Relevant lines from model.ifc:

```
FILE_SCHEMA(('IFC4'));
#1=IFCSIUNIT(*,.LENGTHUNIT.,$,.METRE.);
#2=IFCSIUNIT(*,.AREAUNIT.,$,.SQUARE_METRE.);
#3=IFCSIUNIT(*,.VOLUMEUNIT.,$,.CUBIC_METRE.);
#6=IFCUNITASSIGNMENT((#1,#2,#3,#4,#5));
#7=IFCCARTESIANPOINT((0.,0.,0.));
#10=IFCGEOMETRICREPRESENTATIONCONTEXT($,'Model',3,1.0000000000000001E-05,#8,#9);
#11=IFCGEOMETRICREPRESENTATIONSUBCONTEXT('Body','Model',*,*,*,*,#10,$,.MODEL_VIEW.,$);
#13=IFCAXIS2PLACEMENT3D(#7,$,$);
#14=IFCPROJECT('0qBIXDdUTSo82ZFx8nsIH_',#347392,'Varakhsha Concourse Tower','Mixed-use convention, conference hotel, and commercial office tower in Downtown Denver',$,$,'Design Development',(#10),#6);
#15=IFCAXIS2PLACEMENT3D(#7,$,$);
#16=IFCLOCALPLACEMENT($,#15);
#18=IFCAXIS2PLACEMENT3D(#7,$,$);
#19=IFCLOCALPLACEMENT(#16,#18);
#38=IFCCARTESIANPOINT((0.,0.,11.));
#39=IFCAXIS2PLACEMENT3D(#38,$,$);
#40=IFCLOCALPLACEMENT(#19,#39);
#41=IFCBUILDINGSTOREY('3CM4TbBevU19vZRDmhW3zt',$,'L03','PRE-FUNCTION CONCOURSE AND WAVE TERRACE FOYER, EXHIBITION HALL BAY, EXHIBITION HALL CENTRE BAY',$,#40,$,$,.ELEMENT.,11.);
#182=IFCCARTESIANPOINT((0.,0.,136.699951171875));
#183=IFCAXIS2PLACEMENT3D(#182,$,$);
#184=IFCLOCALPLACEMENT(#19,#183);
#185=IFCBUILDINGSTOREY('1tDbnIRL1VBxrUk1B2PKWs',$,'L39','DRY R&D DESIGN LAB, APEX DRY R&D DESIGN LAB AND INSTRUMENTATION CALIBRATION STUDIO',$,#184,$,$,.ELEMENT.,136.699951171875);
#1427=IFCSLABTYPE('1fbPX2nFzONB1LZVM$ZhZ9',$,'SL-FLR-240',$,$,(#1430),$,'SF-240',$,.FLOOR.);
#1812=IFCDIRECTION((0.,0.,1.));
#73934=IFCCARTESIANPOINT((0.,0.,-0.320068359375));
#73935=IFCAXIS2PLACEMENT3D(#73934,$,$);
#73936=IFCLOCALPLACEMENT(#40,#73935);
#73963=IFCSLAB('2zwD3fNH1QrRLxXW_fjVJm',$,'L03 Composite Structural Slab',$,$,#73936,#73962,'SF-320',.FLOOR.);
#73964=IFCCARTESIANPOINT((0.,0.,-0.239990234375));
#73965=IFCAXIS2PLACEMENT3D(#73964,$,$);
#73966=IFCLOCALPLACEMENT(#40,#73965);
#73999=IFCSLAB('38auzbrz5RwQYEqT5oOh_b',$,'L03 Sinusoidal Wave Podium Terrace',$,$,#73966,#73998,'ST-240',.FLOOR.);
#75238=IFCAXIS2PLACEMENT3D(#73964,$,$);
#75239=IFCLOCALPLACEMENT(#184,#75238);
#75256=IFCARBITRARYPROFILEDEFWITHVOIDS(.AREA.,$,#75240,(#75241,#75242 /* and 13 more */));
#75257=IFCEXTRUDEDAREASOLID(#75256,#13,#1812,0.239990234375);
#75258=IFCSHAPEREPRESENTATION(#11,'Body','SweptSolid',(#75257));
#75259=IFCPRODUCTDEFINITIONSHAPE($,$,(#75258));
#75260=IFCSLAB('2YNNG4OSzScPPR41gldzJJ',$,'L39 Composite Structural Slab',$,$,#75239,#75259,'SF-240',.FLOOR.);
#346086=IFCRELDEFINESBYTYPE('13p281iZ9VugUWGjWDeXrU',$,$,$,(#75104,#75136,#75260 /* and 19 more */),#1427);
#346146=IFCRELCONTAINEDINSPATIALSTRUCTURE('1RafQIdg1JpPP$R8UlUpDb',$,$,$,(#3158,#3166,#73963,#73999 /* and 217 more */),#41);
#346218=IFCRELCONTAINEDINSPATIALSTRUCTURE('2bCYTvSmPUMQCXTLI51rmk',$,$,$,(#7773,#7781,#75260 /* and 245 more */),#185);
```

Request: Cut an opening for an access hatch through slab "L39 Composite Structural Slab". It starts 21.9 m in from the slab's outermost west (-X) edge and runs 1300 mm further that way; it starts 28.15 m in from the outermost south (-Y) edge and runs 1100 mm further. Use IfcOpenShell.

```python
import numpy as np
import ifcopenshell
import ifcopenshell.api.feature
import ifcopenshell.api.geometry
import ifcopenshell.api.root
import ifcopenshell.geom
import ifcopenshell.util.placement
import ifcopenshell.util.representation
import ifcopenshell.util.shape
import ifcopenshell.util.unit

model = ifcopenshell.open("model.ifc")
unit_scale = ifcopenshell.util.unit.calculate_unit_scale(model)
settings = ifcopenshell.geom.settings()


def volume(element):
    """Net volume in cubic metres, openings subtracted."""
    shape = ifcopenshell.geom.create_shape(settings, element)
    return ifcopenshell.util.shape.get_volume(shape.geometry)


slab = model.by_guid("2YNNG4OSzScPPR41gldzJJ")
before = volume(slab)

# Extent in the slab's own axes, in metres. The edges named are its -X and -Y sides.
slab_shape = ifcopenshell.geom.create_shape(settings, slab)
vertices = ifcopenshell.util.shape.get_vertices(slab_shape.geometry)
x_min, y_min, bottom = vertices.min(axis=0)
top = vertices[:, 2].max()

opening = ifcopenshell.api.root.create_entity(model, ifc_class="IfcOpeningElement", name="Access hatch opening", predefined_type="OPENING")
context = ifcopenshell.util.representation.get_context(model, "Model", "Body", "MODEL_VIEW")
width, depth = 1.3, 1.1
outline = [(0.0, 0.0), (width, 0.0), (width, depth), (0.0, depth), (0.0, 0.0)]
# Overshoot both faces by 50 mm so the cut is clean.
shape = ifcopenshell.api.geometry.add_slab_representation(
    model, context=context, depth=top - bottom + 0.1, polyline=outline
)
ifcopenshell.api.geometry.assign_representation(model, product=opening, representation=shape)

matrix = ifcopenshell.util.placement.get_local_placement(slab.ObjectPlacement)
matrix[:, 3] = matrix @ np.append(np.array([x_min + 21.9, y_min + 28.15, bottom - 0.05]) / unit_scale, 1.0)
ifcopenshell.api.geometry.edit_object_placement(model, product=opening, matrix=matrix, is_si=False)
ifcopenshell.api.feature.add_feature(model, feature=opening, element=slab)

after = volume(slab)

print(f"slab volume {before:.3f} -> {after:.3f} m3")

model.write("model_rev.ifc")
```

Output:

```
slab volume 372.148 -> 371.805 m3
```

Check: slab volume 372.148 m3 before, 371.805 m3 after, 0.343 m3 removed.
